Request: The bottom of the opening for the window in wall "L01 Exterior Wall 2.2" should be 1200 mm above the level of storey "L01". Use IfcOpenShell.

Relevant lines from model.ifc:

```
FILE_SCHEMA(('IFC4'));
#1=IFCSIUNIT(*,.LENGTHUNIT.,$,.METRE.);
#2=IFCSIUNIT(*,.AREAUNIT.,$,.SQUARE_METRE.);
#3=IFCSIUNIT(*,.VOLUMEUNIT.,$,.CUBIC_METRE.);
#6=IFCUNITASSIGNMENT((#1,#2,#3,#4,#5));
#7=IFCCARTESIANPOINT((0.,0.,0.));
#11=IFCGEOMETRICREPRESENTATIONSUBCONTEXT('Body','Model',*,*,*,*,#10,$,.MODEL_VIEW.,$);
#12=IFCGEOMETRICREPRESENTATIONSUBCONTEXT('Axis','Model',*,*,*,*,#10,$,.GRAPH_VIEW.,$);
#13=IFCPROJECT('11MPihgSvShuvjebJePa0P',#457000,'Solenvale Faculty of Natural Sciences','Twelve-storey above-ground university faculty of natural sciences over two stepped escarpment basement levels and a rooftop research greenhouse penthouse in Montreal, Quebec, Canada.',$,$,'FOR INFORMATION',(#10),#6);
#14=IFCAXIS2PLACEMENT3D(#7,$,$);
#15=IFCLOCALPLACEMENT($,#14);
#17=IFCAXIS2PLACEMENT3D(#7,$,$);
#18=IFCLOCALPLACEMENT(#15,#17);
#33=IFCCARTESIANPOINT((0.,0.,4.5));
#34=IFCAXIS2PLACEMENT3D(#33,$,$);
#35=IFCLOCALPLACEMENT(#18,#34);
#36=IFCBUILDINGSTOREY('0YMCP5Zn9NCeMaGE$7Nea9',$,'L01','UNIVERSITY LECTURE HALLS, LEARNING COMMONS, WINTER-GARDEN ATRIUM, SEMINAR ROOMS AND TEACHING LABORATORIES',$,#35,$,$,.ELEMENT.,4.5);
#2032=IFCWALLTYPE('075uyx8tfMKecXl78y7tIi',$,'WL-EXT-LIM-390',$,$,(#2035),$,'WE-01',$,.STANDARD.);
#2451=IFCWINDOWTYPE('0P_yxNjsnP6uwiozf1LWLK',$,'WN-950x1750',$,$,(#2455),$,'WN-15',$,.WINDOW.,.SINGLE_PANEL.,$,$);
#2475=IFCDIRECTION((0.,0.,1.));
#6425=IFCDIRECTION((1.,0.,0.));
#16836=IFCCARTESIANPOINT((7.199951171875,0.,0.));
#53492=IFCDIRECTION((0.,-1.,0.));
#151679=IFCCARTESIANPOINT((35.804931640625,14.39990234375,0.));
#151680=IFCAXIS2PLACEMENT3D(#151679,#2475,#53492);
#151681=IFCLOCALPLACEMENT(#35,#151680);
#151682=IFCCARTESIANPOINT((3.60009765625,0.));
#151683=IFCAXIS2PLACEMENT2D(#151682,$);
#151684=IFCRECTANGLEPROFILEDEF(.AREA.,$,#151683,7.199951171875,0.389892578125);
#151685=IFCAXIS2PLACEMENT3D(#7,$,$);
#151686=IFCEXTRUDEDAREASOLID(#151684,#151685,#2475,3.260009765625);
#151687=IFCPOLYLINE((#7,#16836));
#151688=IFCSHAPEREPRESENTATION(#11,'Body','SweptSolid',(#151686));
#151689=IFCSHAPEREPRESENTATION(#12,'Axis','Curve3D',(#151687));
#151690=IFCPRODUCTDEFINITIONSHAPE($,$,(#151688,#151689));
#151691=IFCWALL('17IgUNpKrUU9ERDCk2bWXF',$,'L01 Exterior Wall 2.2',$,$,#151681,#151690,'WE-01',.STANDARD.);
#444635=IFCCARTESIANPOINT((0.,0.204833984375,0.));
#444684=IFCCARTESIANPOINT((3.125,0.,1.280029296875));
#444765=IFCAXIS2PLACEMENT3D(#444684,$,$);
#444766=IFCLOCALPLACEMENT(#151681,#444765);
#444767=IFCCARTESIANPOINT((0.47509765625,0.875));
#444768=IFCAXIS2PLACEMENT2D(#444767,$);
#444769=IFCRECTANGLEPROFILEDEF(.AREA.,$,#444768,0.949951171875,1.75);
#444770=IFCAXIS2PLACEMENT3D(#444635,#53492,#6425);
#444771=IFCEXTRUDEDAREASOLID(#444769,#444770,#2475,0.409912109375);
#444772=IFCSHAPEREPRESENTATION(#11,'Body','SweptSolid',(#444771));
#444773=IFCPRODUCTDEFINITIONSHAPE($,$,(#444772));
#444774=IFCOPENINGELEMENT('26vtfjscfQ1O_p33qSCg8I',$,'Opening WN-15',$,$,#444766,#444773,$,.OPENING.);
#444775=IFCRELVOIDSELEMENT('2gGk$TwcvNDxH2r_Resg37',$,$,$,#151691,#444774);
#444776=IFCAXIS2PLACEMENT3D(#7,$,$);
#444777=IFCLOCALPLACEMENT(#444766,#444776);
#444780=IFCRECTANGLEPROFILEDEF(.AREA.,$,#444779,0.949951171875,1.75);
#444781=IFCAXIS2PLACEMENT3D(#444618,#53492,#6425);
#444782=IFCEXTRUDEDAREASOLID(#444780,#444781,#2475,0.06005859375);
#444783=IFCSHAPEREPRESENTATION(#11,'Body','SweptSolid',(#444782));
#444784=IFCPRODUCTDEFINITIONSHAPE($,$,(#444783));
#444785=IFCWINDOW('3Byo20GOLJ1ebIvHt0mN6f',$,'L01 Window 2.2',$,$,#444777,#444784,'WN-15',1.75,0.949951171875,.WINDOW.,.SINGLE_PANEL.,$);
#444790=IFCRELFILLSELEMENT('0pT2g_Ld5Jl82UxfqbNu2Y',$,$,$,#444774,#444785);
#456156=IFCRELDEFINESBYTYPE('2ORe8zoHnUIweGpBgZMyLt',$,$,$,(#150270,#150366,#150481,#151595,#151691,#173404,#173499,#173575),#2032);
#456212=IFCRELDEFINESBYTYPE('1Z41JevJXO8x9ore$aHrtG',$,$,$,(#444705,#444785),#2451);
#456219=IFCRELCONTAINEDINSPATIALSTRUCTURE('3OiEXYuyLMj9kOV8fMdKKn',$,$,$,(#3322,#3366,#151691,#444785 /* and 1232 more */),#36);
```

```python
import numpy as np
import ifcopenshell
import ifcopenshell.api.geometry
import ifcopenshell.geom
import ifcopenshell.util.element
import ifcopenshell.util.placement
import ifcopenshell.util.shape
import ifcopenshell.util.unit

model = ifcopenshell.open("model.ifc")
unit_scale = ifcopenshell.util.unit.calculate_unit_scale(model)

window = model.by_guid("3Byo20GOLJ1ebIvHt0mN6f")
opening = window.FillsVoids[0].RelatingOpeningElement
storey = ifcopenshell.util.element.get_container(window, ifc_class="IfcBuildingStorey")
level = ifcopenshell.util.placement.get_local_placement(storey.ObjectPlacement)[2, 3]

# The opening's origin need not be at the sill, so measure its lowest point.
shape = ifcopenshell.geom.create_shape(ifcopenshell.geom.settings(), opening)
bottom = ifcopenshell.util.shape.get_shape_bottom_elevation(shape, shape.geometry) / unit_scale
dz = level + 1.2 / unit_scale - bottom

shift = np.array([0.0, 0.0, dz])
# The window is placed relative to its opening, so it follows when the opening moves.
matrix = ifcopenshell.util.placement.get_local_placement(opening.ObjectPlacement)
matrix[:3, 3] += shift
ifcopenshell.api.geometry.edit_object_placement(
    model, product=opening, matrix=matrix, is_si=False, should_transform_children=True
)

print(f"moved by {dz * unit_scale:+.3f} m")

model.write("model_v2.ifc")
```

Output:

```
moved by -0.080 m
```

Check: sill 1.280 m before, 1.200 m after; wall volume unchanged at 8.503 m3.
